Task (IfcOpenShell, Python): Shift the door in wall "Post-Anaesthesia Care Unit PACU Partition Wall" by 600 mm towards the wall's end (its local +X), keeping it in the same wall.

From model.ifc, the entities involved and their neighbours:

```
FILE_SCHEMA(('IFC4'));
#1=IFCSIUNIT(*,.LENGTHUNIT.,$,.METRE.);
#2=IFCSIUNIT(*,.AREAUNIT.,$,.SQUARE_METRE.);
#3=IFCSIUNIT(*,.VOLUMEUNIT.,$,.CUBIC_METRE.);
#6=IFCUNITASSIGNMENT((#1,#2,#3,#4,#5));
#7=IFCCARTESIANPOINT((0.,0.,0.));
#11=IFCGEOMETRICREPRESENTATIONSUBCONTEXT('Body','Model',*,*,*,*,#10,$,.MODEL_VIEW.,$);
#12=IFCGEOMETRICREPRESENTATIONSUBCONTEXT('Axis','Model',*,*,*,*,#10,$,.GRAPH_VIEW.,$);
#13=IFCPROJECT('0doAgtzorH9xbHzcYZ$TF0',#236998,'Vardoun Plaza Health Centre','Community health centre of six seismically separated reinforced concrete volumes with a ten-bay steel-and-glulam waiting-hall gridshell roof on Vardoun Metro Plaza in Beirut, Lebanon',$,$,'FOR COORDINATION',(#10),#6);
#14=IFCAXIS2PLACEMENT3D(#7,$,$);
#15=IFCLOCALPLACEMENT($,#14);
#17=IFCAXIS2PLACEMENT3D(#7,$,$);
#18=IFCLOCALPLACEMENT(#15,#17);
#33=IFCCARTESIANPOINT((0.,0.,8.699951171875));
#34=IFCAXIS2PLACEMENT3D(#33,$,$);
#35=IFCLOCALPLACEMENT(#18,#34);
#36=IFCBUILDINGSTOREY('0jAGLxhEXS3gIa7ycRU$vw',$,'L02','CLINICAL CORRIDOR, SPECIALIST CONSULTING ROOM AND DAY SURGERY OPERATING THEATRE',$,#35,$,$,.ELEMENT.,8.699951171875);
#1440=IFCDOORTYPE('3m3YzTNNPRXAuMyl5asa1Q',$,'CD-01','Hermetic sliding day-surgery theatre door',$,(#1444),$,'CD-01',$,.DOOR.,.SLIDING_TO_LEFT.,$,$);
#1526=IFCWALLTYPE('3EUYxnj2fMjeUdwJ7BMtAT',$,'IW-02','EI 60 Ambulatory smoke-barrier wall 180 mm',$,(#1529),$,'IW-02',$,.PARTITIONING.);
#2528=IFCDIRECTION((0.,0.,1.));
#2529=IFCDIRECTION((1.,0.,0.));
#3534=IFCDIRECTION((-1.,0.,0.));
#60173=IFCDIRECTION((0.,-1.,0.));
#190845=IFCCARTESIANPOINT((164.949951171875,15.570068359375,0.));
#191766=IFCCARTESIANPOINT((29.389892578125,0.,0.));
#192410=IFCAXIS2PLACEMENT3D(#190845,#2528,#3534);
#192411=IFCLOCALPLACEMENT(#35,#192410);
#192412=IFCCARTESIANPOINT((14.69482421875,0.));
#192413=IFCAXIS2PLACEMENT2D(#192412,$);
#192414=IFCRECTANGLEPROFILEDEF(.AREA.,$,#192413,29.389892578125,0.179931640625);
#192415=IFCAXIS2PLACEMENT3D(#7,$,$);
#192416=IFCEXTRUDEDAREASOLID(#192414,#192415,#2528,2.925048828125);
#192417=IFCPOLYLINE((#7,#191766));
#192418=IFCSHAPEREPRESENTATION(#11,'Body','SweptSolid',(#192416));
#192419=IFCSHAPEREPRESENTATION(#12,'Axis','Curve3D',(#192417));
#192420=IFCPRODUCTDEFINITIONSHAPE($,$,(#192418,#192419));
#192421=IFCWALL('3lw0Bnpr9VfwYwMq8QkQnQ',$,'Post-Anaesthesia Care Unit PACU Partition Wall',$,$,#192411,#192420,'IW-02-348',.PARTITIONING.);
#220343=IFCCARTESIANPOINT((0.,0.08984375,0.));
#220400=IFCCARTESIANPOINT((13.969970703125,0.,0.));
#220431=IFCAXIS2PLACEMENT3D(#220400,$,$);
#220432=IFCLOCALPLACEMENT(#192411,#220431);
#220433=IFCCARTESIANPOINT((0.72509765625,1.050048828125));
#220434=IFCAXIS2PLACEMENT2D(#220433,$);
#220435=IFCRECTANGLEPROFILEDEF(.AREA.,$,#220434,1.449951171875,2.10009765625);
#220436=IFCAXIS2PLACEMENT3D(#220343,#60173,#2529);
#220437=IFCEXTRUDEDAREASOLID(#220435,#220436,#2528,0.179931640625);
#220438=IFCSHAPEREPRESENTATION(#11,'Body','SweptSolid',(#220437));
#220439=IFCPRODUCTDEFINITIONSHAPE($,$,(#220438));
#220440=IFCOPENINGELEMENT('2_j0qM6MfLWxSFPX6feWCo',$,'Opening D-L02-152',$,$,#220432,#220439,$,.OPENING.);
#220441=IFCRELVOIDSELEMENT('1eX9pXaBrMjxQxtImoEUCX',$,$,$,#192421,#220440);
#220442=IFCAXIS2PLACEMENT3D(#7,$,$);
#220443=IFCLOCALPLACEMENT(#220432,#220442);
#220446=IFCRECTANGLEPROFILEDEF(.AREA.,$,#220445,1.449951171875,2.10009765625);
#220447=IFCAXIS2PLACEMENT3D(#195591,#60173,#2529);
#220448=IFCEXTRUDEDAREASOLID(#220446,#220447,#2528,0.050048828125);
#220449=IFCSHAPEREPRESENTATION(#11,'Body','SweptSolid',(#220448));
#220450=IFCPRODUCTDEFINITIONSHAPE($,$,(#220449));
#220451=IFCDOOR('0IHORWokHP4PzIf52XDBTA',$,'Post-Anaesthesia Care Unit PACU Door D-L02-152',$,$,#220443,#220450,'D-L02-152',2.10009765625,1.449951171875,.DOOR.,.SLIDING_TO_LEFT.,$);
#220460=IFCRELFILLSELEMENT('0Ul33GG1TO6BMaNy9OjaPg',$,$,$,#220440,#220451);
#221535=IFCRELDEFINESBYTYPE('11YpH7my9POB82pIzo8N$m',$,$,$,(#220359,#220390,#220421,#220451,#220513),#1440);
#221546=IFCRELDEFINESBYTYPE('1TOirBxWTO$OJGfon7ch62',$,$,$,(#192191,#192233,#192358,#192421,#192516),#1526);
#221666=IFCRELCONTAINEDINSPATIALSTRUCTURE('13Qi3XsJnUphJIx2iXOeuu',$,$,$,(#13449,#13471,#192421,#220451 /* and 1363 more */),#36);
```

```python
import ifcopenshell
import ifcopenshell.api.geometry
import ifcopenshell.util.placement

model = ifcopenshell.open("model.ifc")

door = model.by_id(220451)
opening = door.FillsVoids[0].RelatingOpeningElement
wall = opening.VoidsElements[0].RelatingBuildingElement

wall_matrix = ifcopenshell.util.placement.get_local_placement(wall.ObjectPlacement)
shift = wall_matrix[:3, 0] * 0.6
before = ifcopenshell.util.placement.get_local_placement(door.ObjectPlacement)[:3, 3].copy()

# The door is placed relative to its opening, so it follows when the opening moves.
matrix = ifcopenshell.util.placement.get_local_placement(opening.ObjectPlacement)
matrix[:3, 3] += shift
ifcopenshell.api.geometry.edit_object_placement(
    model, product=opening, matrix=matrix, is_si=False, should_transform_children=True
)

after = ifcopenshell.util.placement.get_local_placement(door.ObjectPlacement)[:3, 3]
print("door moved by", (after - before).round(3) + 0.0)

model.write("model_v2.ifc")
```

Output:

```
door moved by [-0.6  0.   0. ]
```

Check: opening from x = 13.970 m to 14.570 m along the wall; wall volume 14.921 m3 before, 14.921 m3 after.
